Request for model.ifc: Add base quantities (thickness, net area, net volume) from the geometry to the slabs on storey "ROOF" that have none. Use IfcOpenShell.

First a look at what the model holds.

```python
import ifcopenshell
import ifcopenshell.util.element
import ifcopenshell.util.unit

model = ifcopenshell.open("model.ifc")
print(model.schema)
for unit_type in ("LENGTHUNIT", "AREAUNIT", "VOLUMEUNIT"):
    print(unit_type, ifcopenshell.util.unit.calculate_unit_scale(model, unit_type))
storey = next(s for s in model.by_type("IfcBuildingStorey") if s.Name == "ROOF")
slabs = [e for e in ifcopenshell.util.element.get_decomposition(storey) if e.is_a("IfcSlab")]
for e in sorted(slabs, key=lambda e: e.id()):
    print(e.id(), e.is_a(), e.Name, list(ifcopenshell.util.element.get_psets(e, qtos_only=True)), sep=" | ")
```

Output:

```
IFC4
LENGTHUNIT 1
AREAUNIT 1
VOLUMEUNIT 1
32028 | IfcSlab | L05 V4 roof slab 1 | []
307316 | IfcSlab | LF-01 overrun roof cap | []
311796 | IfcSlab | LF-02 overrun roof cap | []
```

```python
import ifcopenshell
import ifcopenshell.api.pset
import ifcopenshell.geom
import ifcopenshell.util.element
import ifcopenshell.util.shape
import ifcopenshell.util.unit

model = ifcopenshell.open("model.ifc")
unit_scale = ifcopenshell.util.unit.calculate_unit_scale(model)
area_scale = ifcopenshell.util.unit.calculate_unit_scale(model, "AREAUNIT")
volume_scale = ifcopenshell.util.unit.calculate_unit_scale(model, "VOLUMEUNIT")
settings = ifcopenshell.geom.settings()

storey = next(s for s in model.by_type("IfcBuildingStorey") if s.Name == "ROOF")
slabs = [e for e in ifcopenshell.util.element.get_decomposition(storey) if e.is_a("IfcSlab")]

for e in sorted(slabs, key=lambda e: e.id()):
    if ifcopenshell.util.element.get_psets(e, qtos_only=True, should_inherit=False):
        continue
    # Geometry comes back in metres, in the element's own axes.
    shape = ifcopenshell.geom.create_shape(settings, e)
    values = {
        "Width": ifcopenshell.util.shape.get_z(shape.geometry) / unit_scale,
        "NetArea": ifcopenshell.util.shape.get_footprint_area(shape.geometry) / area_scale,
        "NetVolume": ifcopenshell.util.shape.get_volume(shape.geometry) / volume_scale,
    }
    qto = ifcopenshell.api.pset.add_qto(model, product=e, name="Qto_SlabBaseQuantities")
    ifcopenshell.api.pset.edit_qto(model, qto=qto, properties=values)
    print(e.id(), {k: round(v, 3) for k, v in values.items()})

model.write("model_edited.ifc")
```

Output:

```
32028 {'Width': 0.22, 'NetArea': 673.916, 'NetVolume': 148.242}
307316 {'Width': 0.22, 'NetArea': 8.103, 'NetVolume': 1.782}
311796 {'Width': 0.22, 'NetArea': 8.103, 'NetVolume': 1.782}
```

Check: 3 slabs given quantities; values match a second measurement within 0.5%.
